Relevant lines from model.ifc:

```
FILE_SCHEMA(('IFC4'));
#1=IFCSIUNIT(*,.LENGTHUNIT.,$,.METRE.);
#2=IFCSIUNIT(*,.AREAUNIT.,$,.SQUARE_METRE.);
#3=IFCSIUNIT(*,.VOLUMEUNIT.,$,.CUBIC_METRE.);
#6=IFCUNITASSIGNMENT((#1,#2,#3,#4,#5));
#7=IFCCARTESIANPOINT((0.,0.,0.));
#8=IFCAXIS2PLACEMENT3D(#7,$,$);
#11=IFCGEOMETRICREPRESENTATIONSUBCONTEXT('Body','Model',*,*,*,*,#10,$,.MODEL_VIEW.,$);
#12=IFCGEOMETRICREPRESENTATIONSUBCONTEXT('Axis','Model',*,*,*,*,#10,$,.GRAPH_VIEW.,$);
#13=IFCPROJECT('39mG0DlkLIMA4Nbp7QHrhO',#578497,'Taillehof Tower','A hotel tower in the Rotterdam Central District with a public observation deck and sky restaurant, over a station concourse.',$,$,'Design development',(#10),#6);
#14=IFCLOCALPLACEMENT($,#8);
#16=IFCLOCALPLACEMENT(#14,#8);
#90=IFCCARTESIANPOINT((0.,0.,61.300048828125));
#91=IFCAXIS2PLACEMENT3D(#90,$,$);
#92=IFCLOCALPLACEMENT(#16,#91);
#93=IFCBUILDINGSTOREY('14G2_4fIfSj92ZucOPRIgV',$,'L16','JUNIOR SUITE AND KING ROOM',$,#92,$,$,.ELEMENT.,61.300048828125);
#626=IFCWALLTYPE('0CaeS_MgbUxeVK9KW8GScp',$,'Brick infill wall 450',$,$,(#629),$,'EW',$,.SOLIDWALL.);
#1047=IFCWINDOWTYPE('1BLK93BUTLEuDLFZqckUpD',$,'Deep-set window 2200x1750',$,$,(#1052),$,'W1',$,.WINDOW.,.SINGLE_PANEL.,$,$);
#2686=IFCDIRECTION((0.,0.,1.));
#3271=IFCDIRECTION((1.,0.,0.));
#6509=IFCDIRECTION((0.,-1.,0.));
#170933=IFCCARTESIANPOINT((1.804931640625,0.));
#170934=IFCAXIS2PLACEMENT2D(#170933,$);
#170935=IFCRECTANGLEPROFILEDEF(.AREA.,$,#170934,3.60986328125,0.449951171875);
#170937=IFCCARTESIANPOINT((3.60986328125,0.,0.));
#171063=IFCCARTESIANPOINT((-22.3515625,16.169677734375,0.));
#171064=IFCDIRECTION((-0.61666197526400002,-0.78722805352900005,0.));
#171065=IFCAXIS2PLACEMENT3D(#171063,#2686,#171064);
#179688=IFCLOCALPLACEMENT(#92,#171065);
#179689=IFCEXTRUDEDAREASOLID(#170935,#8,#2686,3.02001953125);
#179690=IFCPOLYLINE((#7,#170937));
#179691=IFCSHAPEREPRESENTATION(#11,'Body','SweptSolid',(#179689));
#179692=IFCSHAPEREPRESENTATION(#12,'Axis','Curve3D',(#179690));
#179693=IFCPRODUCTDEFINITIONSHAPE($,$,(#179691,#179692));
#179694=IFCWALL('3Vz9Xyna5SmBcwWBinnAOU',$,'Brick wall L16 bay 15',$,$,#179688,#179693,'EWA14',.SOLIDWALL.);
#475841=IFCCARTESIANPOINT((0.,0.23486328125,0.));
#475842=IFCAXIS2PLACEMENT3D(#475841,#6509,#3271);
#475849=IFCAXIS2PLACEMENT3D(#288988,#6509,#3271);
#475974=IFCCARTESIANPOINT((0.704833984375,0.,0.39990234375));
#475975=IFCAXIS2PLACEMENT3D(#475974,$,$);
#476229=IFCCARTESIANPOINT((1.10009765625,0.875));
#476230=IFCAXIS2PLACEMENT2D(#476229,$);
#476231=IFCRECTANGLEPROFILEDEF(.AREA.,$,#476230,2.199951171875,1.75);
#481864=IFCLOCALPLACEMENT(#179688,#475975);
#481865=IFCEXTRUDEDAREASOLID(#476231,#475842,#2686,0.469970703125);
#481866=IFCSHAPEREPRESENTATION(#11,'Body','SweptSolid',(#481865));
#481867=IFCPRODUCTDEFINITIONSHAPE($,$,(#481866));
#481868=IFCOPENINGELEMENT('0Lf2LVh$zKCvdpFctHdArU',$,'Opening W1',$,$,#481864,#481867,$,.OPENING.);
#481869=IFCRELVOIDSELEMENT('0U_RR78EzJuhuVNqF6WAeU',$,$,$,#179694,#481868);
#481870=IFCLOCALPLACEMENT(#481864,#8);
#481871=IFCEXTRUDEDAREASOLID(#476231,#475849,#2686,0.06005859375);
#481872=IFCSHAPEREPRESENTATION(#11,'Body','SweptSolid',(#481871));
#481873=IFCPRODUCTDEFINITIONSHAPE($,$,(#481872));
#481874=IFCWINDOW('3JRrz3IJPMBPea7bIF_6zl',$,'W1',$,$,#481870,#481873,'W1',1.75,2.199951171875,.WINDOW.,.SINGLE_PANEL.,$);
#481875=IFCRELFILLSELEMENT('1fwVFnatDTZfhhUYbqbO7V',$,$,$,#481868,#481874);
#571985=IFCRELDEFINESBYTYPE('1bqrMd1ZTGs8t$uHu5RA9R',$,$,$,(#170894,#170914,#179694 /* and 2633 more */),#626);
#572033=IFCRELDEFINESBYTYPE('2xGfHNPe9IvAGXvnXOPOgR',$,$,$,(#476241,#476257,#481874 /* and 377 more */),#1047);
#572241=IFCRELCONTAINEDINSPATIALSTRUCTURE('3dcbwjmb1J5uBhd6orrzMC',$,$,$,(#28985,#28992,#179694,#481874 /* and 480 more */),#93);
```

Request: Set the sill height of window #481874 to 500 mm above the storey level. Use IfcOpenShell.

```python
import numpy as np
import ifcopenshell
import ifcopenshell.api.geometry
import ifcopenshell.geom
import ifcopenshell.util.element
import ifcopenshell.util.placement
import ifcopenshell.util.shape
import ifcopenshell.util.unit

model = ifcopenshell.open("model.ifc")
unit_scale = ifcopenshell.util.unit.calculate_unit_scale(model)

window = model.by_guid("3JRrz3IJPMBPea7bIF_6zl")
opening = window.FillsVoids[0].RelatingOpeningElement
storey = ifcopenshell.util.element.get_container(window, ifc_class="IfcBuildingStorey")
level = ifcopenshell.util.placement.get_local_placement(storey.ObjectPlacement)[2, 3]

# The opening's origin need not be at the sill, so measure its lowest point.
shape = ifcopenshell.geom.create_shape(ifcopenshell.geom.settings(), opening)
bottom = ifcopenshell.util.shape.get_shape_bottom_elevation(shape, shape.geometry) / unit_scale
dz = level + 0.5 / unit_scale - bottom

shift = np.array([0.0, 0.0, dz])
# The window is placed relative to its opening, so it follows when the opening moves.
matrix = ifcopenshell.util.placement.get_local_placement(opening.ObjectPlacement)
matrix[:3, 3] += shift
ifcopenshell.api.geometry.edit_object_placement(
    model, product=opening, matrix=matrix, is_si=False, should_transform_children=True
)

print(f"moved by {dz * unit_scale:+.3f} m")

model.write("model_v2.ifc")
```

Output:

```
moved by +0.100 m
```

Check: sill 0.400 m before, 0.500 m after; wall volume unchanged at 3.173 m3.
